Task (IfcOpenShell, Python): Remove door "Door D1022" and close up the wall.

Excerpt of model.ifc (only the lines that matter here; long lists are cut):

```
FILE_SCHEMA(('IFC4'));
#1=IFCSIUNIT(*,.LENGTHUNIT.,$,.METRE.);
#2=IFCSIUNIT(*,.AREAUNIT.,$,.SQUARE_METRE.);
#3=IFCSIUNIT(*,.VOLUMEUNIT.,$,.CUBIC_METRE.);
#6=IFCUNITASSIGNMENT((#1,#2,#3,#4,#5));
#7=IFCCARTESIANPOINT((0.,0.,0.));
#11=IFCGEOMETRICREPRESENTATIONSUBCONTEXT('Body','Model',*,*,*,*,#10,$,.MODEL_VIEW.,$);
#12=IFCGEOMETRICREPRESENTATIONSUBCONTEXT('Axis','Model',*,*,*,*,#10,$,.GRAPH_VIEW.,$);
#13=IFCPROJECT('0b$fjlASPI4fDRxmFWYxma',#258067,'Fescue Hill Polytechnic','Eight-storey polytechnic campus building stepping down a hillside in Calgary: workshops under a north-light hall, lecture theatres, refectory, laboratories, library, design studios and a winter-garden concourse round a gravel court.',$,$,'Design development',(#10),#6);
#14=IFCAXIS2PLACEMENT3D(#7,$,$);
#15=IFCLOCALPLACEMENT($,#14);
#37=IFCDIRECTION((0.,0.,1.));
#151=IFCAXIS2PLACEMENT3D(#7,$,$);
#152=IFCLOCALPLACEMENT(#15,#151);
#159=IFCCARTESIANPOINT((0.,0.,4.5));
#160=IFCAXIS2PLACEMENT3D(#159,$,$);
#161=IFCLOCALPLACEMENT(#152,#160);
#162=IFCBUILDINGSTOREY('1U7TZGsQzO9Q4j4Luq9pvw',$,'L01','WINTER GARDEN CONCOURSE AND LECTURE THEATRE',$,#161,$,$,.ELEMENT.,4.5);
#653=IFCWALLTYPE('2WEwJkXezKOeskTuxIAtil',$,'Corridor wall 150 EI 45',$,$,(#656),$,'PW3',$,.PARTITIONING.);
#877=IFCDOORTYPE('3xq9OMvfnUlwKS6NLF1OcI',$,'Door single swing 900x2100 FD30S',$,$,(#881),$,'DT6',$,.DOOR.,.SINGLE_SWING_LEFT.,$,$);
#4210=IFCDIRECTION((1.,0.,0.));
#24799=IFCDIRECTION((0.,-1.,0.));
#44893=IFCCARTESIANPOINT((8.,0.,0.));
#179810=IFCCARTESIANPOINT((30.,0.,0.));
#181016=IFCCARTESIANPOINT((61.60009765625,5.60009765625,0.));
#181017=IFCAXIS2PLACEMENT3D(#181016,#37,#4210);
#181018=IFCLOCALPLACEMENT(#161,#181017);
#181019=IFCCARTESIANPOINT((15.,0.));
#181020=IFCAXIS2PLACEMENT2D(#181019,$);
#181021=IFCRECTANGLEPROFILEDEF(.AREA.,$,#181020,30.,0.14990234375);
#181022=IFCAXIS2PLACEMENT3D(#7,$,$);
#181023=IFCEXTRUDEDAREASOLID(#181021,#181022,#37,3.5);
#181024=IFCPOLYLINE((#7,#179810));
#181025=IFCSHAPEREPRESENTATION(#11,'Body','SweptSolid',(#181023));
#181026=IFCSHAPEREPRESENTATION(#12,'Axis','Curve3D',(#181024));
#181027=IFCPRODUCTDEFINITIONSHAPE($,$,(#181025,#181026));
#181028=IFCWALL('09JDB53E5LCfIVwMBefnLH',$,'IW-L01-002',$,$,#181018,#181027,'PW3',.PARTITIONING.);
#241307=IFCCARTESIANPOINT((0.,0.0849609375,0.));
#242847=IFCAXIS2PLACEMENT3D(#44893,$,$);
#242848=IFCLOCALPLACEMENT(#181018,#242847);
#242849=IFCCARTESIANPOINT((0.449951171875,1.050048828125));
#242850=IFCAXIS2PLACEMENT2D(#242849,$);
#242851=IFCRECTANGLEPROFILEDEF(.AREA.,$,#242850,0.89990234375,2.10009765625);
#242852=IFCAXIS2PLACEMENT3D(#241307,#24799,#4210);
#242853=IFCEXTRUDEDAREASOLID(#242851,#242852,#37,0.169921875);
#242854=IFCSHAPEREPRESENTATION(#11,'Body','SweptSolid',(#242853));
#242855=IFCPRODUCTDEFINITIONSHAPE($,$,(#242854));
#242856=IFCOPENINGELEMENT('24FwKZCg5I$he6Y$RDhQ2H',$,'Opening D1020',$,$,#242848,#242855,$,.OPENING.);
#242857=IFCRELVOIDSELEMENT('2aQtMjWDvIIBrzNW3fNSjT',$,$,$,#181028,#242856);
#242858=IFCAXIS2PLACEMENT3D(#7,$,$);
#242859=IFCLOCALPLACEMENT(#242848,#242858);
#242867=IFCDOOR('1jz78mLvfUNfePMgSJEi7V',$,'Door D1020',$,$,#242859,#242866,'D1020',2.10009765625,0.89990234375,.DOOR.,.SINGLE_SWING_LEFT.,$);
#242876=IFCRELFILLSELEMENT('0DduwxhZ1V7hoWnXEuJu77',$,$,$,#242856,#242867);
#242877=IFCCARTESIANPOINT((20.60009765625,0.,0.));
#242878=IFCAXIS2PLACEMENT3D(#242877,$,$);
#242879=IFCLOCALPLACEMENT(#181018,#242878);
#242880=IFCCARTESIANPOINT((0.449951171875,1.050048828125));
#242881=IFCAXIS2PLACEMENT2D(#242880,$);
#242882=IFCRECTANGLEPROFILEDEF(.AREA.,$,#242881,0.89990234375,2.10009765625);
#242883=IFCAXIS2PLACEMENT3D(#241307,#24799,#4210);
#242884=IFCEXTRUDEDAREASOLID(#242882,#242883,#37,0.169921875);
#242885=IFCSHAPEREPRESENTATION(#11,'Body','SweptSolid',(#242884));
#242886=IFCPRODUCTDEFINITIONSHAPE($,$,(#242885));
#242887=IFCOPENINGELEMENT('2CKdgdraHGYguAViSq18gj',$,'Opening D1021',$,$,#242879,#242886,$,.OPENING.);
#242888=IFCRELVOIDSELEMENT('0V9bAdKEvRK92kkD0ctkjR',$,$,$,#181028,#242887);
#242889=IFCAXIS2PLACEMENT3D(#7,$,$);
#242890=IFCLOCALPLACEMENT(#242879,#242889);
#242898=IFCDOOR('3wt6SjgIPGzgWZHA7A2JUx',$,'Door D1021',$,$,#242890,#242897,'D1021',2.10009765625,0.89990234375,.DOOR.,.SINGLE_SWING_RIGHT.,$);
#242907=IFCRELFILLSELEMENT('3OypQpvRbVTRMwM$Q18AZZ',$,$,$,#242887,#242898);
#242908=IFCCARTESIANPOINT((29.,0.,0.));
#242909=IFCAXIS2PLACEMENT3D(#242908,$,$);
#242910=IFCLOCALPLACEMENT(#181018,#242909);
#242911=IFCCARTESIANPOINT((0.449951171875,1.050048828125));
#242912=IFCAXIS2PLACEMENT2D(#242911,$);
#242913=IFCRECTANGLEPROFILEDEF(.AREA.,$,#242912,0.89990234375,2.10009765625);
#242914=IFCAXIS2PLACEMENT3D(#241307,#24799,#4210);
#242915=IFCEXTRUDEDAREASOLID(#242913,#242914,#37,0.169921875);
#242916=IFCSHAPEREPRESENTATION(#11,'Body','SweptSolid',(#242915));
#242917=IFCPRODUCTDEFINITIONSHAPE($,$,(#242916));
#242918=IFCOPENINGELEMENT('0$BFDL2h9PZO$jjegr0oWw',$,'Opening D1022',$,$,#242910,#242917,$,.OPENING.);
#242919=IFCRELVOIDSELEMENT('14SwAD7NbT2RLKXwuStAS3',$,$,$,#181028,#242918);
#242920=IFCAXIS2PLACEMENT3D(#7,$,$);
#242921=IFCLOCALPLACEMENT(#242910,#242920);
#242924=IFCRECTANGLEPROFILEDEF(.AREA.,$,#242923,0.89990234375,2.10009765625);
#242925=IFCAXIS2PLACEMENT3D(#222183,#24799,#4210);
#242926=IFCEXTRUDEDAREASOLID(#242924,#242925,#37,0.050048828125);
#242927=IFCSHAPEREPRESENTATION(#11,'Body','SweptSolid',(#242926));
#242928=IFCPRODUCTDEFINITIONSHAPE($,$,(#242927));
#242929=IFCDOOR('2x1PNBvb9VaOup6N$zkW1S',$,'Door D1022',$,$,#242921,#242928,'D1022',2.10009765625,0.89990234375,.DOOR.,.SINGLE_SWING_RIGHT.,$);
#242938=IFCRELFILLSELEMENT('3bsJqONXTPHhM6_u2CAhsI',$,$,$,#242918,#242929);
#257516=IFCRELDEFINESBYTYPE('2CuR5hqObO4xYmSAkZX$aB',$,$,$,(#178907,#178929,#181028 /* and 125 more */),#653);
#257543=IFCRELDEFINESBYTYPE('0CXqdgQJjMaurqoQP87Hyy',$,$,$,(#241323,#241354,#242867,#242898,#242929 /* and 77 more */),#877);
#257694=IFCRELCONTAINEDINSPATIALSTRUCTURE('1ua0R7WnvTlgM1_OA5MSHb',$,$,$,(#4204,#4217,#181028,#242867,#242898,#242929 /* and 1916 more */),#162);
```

```python
import ifcopenshell
import ifcopenshell.api.feature
import ifcopenshell.api.root
import ifcopenshell.geom
import ifcopenshell.util.shape

model = ifcopenshell.open("model.ifc")
settings = ifcopenshell.geom.settings()


def volume(element):
    """Net volume in cubic metres, openings subtracted."""
    shape = ifcopenshell.geom.create_shape(settings, element)
    return ifcopenshell.util.shape.get_volume(shape.geometry)


door = model.by_id(242929)
opening = door.FillsVoids[0].RelatingOpeningElement
wall = opening.VoidsElements[0].RelatingBuildingElement
before = volume(wall)

ifcopenshell.api.root.remove_product(model, product=door)
ifcopenshell.api.feature.remove_feature(model, feature=opening)

after = volume(wall)

print(f"wall volume {before:.3f} -> {after:.3f} m3")

model.write("model_edited.ifc")
```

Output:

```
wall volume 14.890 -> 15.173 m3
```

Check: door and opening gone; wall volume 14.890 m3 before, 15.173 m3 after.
